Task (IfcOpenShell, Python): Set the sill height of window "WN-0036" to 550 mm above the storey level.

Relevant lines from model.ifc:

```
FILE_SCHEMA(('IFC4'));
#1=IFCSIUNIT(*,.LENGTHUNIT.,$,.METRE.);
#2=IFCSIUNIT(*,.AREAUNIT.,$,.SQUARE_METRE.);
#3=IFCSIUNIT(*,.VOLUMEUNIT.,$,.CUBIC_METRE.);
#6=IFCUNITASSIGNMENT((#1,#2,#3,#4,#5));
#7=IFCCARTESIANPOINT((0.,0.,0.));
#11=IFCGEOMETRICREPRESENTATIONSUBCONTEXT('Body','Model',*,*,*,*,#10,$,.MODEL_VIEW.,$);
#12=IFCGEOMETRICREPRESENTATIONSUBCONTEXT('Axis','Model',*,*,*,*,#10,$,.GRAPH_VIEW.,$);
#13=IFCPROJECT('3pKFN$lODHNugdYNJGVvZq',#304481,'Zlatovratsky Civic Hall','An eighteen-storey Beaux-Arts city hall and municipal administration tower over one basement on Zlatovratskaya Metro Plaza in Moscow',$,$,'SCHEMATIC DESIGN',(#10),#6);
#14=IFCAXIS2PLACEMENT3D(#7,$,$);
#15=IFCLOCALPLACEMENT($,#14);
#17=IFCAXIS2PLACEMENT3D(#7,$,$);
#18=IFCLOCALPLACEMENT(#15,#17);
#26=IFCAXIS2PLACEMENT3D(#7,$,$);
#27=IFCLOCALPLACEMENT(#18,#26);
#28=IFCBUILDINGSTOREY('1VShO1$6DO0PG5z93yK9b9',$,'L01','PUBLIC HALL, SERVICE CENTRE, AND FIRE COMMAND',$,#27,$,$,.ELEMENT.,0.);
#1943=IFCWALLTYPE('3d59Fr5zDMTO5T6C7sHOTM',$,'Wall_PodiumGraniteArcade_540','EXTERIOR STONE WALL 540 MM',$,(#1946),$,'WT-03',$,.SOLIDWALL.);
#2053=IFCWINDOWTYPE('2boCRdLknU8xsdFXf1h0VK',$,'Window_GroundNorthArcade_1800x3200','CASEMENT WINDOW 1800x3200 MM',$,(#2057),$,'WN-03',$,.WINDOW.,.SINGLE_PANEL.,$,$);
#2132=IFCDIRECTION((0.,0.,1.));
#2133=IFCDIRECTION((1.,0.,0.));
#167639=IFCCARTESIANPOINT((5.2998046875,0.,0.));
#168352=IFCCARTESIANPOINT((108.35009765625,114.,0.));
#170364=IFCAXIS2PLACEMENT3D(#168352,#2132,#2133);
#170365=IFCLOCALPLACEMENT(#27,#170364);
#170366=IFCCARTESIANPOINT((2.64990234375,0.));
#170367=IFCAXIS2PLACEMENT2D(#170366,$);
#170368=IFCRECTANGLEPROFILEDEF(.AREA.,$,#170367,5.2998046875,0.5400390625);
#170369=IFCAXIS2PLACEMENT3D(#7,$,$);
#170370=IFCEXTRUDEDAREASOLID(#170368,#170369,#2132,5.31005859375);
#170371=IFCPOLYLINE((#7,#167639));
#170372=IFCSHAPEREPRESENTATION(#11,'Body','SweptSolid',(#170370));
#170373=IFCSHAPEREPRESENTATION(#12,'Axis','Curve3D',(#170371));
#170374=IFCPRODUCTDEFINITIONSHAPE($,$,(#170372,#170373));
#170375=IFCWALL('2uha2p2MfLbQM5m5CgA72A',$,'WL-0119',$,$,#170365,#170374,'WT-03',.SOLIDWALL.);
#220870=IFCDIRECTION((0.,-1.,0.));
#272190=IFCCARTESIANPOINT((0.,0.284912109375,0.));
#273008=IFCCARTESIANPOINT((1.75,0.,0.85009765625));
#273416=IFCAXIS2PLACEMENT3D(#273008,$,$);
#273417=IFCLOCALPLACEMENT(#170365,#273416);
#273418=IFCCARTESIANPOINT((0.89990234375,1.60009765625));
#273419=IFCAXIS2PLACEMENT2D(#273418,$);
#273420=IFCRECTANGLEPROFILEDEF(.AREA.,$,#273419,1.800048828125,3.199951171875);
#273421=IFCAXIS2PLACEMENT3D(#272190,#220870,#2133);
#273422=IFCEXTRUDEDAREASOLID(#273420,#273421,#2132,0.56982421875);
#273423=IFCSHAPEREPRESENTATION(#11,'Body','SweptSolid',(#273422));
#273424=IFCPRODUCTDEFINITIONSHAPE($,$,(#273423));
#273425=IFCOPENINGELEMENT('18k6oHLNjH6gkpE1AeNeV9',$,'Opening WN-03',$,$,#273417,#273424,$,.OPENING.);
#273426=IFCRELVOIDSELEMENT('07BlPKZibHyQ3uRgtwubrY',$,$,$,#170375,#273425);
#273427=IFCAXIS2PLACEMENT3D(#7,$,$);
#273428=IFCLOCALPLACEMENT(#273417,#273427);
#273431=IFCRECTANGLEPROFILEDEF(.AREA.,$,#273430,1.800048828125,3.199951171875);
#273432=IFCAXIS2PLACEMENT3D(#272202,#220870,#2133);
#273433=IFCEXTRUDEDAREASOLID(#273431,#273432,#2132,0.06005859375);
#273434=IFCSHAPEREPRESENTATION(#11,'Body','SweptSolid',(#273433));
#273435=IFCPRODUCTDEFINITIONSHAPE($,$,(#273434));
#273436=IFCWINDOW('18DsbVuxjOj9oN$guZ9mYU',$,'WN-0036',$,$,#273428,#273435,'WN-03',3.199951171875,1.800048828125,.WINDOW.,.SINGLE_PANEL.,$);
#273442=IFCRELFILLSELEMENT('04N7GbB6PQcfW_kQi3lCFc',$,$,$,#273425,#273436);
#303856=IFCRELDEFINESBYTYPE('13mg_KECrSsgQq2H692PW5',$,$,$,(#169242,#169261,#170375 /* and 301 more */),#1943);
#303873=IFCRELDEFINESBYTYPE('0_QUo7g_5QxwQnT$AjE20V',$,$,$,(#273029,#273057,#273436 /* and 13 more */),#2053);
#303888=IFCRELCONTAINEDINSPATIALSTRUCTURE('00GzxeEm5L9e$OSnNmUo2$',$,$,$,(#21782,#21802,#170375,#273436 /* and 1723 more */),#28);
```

```python
import numpy as np
import ifcopenshell
import ifcopenshell.api.geometry
import ifcopenshell.geom
import ifcopenshell.util.element
import ifcopenshell.util.placement
import ifcopenshell.util.shape
import ifcopenshell.util.unit

model = ifcopenshell.open("model.ifc")
unit_scale = ifcopenshell.util.unit.calculate_unit_scale(model)

window = model.by_id(273436)
opening = window.FillsVoids[0].RelatingOpeningElement
storey = ifcopenshell.util.element.get_container(window, ifc_class="IfcBuildingStorey")
level = ifcopenshell.util.placement.get_local_placement(storey.ObjectPlacement)[2, 3]

# The opening's origin need not be at the sill, so measure its lowest point.
shape = ifcopenshell.geom.create_shape(ifcopenshell.geom.settings(), opening)
bottom = ifcopenshell.util.shape.get_shape_bottom_elevation(shape, shape.geometry) / unit_scale
dz = level + 0.55 / unit_scale - bottom

shift = np.array([0.0, 0.0, dz])
# The window is placed relative to its opening, so it follows when the opening moves.
matrix = ifcopenshell.util.placement.get_local_placement(opening.ObjectPlacement)
matrix[:3, 3] += shift
ifcopenshell.api.geometry.edit_object_placement(
    model, product=opening, matrix=matrix, is_si=False, should_transform_children=True
)

print(f"moved by {dz * unit_scale:+.3f} m")

model.write("model-out.ifc")
```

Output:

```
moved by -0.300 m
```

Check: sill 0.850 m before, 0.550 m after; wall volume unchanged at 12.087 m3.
